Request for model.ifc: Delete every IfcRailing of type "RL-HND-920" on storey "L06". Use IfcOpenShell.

First a look at what the model holds.

```python
import ifcopenshell
import ifcopenshell.util.element

model = ifcopenshell.open("model.ifc")
print(model.schema)
storey = next(s for s in model.by_type("IfcBuildingStorey") if s.Name == "L06")
railings = [e for e in ifcopenshell.util.element.get_decomposition(storey) if e.is_a("IfcRailing")]
seen = {}
for e in railings:
    element_type = ifcopenshell.util.element.get_type(e)
    name = element_type.Name if element_type not in (None, e) else None
    seen[name] = seen.get(name, 0) + 1
for name, count in sorted(seen.items(), key=str):
    print(count, "x", name)
```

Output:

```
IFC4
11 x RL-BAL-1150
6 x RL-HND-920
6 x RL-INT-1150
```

```python
import ifcopenshell
import ifcopenshell.api.root
import ifcopenshell.util.element

model = ifcopenshell.open("model.ifc")

storey = next(s for s in model.by_type("IfcBuildingStorey") if s.Name == "L06")
railings = [e for e in ifcopenshell.util.element.get_decomposition(storey) if e.is_a("IfcRailing")]
targets = [e for e in railings if (t := ifcopenshell.util.element.get_type(e)) not in (None, e) and t.Name == "RL-HND-920"]

for e in targets:
    ifcopenshell.api.root.remove_product(model, product=e)
print(len(targets), "removed")

model.write("model_rev.ifc")
```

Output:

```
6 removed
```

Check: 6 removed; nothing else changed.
